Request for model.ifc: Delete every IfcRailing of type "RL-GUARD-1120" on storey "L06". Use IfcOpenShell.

First a look at what the model holds.

```python
import ifcopenshell
import ifcopenshell.util.element

model = ifcopenshell.open("model.ifc")
print(model.schema)
storey = next(s for s in model.by_type("IfcBuildingStorey") if s.Name == "L06")
railings = [e for e in ifcopenshell.util.element.get_decomposition(storey) if e.is_a("IfcRailing")]
seen = {}
for e in railings:
    element_type = ifcopenshell.util.element.get_type(e)
    name = element_type.Name if element_type not in (None, e) else None
    seen[name] = seen.get(name, 0) + 1
for name, count in sorted(seen.items(), key=str):
    print(count, "x", name)
```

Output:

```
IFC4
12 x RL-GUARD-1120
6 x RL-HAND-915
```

```python
import ifcopenshell
import ifcopenshell.api.root
import ifcopenshell.util.element

model = ifcopenshell.open("model.ifc")

storey = next(s for s in model.by_type("IfcBuildingStorey") if s.Name == "L06")
railings = [e for e in ifcopenshell.util.element.get_decomposition(storey) if e.is_a("IfcRailing")]
targets = [e for e in railings if (t := ifcopenshell.util.element.get_type(e)) not in (None, e) and t.Name == "RL-GUARD-1120"]

for e in targets:
    ifcopenshell.api.root.remove_product(model, product=e)
print(len(targets), "removed")

model.write("model_v2.ifc")
```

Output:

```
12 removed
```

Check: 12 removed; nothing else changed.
